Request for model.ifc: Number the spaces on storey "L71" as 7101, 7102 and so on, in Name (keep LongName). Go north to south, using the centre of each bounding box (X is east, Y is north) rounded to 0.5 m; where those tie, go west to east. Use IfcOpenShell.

First a look at what the model holds.

```python
import ifcopenshell
import ifcopenshell.util.element
import ifcopenshell.util.placement

model = ifcopenshell.open("model.ifc")
print(model.schema)
storey = next(s for s in model.by_type("IfcBuildingStorey") if s.Name == "L71")
spaces = [e for e in ifcopenshell.util.element.get_decomposition(storey) if e.is_a("IfcSpace")]
for e in sorted(spaces, key=lambda e: e.id()):
    origin = ifcopenshell.util.placement.get_local_placement(e.ObjectPlacement)[:3, 3]
    print(e.id(), e.Name, e.LongName, origin.round(2) + 0.0, sep=" | ")
```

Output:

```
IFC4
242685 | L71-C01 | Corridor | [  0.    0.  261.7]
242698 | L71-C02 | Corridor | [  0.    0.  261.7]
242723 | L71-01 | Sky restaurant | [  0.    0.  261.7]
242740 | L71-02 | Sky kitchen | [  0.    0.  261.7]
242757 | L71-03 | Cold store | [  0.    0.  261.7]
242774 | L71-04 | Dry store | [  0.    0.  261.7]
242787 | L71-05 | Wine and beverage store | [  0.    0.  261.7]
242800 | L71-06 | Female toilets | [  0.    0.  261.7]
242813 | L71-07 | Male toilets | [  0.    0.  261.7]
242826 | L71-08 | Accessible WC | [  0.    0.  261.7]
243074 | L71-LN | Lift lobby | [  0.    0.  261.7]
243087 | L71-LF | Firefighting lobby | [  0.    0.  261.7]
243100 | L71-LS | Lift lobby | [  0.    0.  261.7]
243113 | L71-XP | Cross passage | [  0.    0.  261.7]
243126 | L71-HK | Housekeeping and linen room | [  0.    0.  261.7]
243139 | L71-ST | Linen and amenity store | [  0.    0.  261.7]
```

```python
import ifcopenshell
import ifcopenshell.geom
import ifcopenshell.util.element
import ifcopenshell.util.shape

model = ifcopenshell.open("model.ifc")
settings = ifcopenshell.geom.settings()
settings.set("use-world-coords", True)


def centre(element):
    shape = ifcopenshell.geom.create_shape(settings, element)
    return ifcopenshell.util.shape.get_bbox_centroid(shape.geometry)


storey = next(s for s in model.by_type("IfcBuildingStorey") if s.Name == "L71")
spaces = [e for e in ifcopenshell.util.element.get_decomposition(storey) if e.is_a("IfcSpace")]

# Insertion points can sit at a corner or the storey origin, so sort by the geometry (in metres).
centres = {e: centre(e) for e in spaces}
spaces.sort(key=lambda e: (-round(centres[e][1] / 0.5), centres[e][0]))

for i, e in enumerate(spaces, start=1):
    number = f"71{i:02d}"
    e.Name = number
    print(e.id(), number)

model.write("model_edited.ifc")
```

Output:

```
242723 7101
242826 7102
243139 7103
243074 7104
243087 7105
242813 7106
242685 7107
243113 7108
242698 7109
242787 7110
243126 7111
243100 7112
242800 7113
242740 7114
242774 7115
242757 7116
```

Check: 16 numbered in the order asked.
